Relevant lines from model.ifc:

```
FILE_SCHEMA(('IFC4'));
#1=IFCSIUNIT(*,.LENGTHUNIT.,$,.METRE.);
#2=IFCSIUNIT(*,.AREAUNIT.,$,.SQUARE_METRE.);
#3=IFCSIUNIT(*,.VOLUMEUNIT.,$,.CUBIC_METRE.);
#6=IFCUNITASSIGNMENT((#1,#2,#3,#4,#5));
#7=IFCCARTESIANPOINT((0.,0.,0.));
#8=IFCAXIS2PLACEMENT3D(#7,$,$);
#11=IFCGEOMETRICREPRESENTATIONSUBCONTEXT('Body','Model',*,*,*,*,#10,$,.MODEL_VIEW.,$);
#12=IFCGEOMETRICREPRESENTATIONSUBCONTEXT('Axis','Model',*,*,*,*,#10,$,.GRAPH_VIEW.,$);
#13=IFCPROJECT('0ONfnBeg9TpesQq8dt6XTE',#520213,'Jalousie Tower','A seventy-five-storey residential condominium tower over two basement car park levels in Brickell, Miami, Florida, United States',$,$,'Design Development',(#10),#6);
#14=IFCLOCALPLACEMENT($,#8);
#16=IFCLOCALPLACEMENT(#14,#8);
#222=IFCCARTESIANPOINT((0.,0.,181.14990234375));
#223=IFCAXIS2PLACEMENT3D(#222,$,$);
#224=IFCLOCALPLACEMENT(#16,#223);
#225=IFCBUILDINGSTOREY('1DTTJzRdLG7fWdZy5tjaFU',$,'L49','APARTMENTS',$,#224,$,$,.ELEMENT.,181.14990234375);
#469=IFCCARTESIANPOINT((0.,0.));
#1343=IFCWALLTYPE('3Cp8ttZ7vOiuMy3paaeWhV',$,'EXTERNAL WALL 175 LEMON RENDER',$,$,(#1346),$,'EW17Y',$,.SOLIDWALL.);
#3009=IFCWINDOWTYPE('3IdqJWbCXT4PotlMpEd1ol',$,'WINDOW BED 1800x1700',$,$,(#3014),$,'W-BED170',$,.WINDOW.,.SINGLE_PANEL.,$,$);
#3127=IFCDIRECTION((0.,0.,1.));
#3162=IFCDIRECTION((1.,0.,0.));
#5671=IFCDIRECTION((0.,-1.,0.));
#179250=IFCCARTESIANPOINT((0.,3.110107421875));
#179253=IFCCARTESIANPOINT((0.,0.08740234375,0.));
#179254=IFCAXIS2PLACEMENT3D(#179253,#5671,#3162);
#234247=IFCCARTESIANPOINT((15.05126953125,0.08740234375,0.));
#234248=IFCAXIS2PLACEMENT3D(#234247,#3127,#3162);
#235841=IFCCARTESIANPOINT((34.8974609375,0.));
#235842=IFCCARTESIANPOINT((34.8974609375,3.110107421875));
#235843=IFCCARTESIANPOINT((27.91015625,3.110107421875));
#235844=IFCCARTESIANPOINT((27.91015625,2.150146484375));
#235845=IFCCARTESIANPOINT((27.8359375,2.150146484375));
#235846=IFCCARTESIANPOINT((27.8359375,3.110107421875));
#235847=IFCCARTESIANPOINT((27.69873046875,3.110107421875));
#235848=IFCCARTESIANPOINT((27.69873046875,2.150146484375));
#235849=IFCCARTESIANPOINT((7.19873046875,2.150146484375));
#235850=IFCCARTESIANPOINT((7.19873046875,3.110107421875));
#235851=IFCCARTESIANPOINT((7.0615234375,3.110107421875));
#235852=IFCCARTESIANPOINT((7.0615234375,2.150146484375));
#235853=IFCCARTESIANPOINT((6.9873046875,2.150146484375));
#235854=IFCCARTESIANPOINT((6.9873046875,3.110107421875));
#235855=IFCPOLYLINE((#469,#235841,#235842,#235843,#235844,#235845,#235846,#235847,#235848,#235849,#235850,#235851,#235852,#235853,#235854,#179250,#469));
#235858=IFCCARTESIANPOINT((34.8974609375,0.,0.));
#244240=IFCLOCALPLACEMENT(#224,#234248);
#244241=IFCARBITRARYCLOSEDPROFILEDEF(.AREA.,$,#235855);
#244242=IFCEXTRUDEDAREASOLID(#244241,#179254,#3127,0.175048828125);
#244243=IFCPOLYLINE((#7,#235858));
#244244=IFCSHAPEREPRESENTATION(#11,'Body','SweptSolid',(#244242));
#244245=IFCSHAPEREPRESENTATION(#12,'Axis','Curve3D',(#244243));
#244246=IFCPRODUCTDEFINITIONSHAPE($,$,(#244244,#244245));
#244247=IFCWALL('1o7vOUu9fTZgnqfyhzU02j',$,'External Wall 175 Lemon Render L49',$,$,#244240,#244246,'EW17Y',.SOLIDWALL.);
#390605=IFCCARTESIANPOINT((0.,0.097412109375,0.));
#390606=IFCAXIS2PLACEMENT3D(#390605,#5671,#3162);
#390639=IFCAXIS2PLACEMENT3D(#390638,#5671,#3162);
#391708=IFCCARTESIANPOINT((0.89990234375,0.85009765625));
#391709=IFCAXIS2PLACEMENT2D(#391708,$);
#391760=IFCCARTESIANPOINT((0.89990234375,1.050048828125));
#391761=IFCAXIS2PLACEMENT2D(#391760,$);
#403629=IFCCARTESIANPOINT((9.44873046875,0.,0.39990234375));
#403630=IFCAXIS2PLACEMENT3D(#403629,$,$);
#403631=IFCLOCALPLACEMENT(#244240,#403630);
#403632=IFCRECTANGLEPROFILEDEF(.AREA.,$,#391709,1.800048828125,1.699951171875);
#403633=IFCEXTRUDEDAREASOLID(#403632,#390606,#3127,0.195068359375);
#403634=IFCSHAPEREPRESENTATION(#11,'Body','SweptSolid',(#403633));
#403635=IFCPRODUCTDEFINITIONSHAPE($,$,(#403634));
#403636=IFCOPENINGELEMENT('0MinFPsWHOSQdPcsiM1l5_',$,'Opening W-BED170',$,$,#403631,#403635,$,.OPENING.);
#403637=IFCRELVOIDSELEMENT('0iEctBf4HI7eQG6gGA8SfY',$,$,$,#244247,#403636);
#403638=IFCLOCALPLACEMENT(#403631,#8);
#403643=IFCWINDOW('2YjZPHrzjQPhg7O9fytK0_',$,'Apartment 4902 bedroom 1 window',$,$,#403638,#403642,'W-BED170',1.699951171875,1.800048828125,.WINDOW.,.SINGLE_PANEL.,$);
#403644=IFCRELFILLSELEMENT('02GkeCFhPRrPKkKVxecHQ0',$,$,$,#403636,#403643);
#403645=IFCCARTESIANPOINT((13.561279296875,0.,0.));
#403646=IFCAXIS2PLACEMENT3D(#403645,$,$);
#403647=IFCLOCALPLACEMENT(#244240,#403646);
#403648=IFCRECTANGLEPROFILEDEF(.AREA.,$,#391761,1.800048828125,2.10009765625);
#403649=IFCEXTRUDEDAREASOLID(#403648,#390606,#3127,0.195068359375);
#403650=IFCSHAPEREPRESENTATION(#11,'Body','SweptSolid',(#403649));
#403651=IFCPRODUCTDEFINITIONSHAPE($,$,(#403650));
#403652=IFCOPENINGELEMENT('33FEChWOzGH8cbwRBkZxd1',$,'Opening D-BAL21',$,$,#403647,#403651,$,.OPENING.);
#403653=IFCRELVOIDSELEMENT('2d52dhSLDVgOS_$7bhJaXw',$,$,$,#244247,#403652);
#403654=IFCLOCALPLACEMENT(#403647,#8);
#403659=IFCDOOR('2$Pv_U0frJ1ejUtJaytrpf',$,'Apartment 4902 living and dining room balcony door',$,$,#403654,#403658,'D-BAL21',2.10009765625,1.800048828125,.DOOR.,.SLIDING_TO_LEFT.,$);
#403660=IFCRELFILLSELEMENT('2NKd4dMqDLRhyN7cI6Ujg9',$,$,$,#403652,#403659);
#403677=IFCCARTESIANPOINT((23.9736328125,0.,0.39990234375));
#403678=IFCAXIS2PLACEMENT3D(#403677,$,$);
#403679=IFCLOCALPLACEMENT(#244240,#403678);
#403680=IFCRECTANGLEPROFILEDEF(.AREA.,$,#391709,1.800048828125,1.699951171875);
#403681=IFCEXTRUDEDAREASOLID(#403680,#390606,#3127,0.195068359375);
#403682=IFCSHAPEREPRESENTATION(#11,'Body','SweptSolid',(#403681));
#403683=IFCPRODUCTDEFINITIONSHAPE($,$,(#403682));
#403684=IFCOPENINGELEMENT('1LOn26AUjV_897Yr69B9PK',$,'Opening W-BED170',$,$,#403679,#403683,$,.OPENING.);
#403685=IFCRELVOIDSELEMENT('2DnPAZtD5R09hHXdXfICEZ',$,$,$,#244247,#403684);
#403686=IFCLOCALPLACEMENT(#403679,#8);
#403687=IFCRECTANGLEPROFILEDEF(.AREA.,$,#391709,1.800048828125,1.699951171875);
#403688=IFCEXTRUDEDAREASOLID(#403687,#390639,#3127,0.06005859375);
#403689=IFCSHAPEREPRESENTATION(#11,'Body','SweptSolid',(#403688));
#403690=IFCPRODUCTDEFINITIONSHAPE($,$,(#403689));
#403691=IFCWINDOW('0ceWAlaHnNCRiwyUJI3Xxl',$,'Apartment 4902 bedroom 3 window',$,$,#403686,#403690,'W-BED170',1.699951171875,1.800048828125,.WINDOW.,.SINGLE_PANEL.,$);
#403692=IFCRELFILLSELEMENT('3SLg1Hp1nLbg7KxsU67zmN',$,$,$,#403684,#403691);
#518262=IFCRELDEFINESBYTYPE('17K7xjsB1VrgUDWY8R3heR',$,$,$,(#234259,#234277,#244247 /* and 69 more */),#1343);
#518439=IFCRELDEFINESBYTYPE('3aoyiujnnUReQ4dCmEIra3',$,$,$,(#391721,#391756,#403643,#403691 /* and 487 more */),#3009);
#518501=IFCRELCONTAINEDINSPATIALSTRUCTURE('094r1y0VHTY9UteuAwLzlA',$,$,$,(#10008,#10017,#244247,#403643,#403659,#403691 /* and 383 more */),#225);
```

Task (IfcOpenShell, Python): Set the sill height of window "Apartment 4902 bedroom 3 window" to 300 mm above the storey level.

```python
import numpy as np
import ifcopenshell
import ifcopenshell.api.geometry
import ifcopenshell.geom
import ifcopenshell.util.element
import ifcopenshell.util.placement
import ifcopenshell.util.shape
import ifcopenshell.util.unit

model = ifcopenshell.open("model.ifc")
unit_scale = ifcopenshell.util.unit.calculate_unit_scale(model)

window = model.by_id(403691)
opening = window.FillsVoids[0].RelatingOpeningElement
storey = ifcopenshell.util.element.get_container(window, ifc_class="IfcBuildingStorey")
level = ifcopenshell.util.placement.get_local_placement(storey.ObjectPlacement)[2, 3]

# The opening's origin need not be at the sill, so measure its lowest point.
shape = ifcopenshell.geom.create_shape(ifcopenshell.geom.settings(), opening)
bottom = ifcopenshell.util.shape.get_shape_bottom_elevation(shape, shape.geometry) / unit_scale
dz = level + 0.3 / unit_scale - bottom

shift = np.array([0.0, 0.0, dz])
# The window is placed relative to its opening, so it follows when the opening moves.
matrix = ifcopenshell.util.placement.get_local_placement(opening.ObjectPlacement)
matrix[:3, 3] += shift
ifcopenshell.api.geometry.edit_object_placement(
    model, product=opening, matrix=matrix, is_si=False, should_transform_children=True
)

print(f"moved by {dz * unit_scale:+.3f} m")

model.write("model_updated.ifc")
```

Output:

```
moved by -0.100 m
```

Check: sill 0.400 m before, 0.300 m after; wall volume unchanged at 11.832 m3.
